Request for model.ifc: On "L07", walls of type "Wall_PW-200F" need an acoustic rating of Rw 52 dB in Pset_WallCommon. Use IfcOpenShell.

First a look at what the model holds.

```python
import ifcopenshell
import ifcopenshell.util.element

model = ifcopenshell.open("model.ifc")
print(model.schema)
storey = next(s for s in model.by_type("IfcBuildingStorey") if s.Name == "L07")
walls = [e for e in ifcopenshell.util.element.get_decomposition(storey) if e.is_a("IfcWall")]
seen = {}
for e in walls:
    element_type = ifcopenshell.util.element.get_type(e)
    key = (element_type.Name if element_type != e and element_type else None, ifcopenshell.util.element.get_pset(e, "Pset_WallCommon", "AcousticRating"))
    seen[key] = seen.get(key, 0) + 1
for (name, value), count in sorted(seen.items(), key=str):
    print(count, "x", name, "|", value)
```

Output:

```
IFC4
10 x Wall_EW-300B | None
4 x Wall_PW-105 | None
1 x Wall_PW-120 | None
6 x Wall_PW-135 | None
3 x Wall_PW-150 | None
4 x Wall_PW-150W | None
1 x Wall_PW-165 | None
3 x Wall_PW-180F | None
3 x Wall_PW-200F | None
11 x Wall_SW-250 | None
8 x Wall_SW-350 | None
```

```python
import ifcopenshell
import ifcopenshell.api.pset
import ifcopenshell.util.element

model = ifcopenshell.open("model.ifc")

storey = next(s for s in model.by_type("IfcBuildingStorey") if s.Name == "L07")
walls = [e for e in ifcopenshell.util.element.get_decomposition(storey) if e.is_a("IfcWall")]

count = 0
for e in walls:
    element_type = ifcopenshell.util.element.get_type(e)
    if element_type in (None, e) or element_type.Name != "Wall_PW-200F":
        continue
    # add_pset returns the element's existing set when there is one.
    pset = ifcopenshell.api.pset.add_pset(model, product=e, name="Pset_WallCommon")
    ifcopenshell.api.pset.edit_pset(model, pset=pset, properties={"AcousticRating": "Rw 52 dB"})
    count += 1

print(count, "walls updated")

model.write("model-out.ifc")
```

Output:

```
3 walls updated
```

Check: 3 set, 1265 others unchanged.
